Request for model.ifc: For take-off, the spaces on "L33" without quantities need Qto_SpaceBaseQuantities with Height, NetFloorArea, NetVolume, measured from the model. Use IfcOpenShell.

First a look at what the model holds.

```python
import ifcopenshell
import ifcopenshell.util.element
import ifcopenshell.util.unit

model = ifcopenshell.open("model.ifc")
print(model.schema)
for unit_type in ("LENGTHUNIT", "AREAUNIT", "VOLUMEUNIT"):
    print(unit_type, ifcopenshell.util.unit.calculate_unit_scale(model, unit_type))
storey = next(s for s in model.by_type("IfcBuildingStorey") if s.Name == "L33")
spaces = [e for e in ifcopenshell.util.element.get_decomposition(storey) if e.is_a("IfcSpace")]
for e in sorted(spaces, key=lambda e: e.id()):
    print(e.id(), e.is_a(), e.Name, list(ifcopenshell.util.element.get_psets(e, qtos_only=True)), sep=" | ")
```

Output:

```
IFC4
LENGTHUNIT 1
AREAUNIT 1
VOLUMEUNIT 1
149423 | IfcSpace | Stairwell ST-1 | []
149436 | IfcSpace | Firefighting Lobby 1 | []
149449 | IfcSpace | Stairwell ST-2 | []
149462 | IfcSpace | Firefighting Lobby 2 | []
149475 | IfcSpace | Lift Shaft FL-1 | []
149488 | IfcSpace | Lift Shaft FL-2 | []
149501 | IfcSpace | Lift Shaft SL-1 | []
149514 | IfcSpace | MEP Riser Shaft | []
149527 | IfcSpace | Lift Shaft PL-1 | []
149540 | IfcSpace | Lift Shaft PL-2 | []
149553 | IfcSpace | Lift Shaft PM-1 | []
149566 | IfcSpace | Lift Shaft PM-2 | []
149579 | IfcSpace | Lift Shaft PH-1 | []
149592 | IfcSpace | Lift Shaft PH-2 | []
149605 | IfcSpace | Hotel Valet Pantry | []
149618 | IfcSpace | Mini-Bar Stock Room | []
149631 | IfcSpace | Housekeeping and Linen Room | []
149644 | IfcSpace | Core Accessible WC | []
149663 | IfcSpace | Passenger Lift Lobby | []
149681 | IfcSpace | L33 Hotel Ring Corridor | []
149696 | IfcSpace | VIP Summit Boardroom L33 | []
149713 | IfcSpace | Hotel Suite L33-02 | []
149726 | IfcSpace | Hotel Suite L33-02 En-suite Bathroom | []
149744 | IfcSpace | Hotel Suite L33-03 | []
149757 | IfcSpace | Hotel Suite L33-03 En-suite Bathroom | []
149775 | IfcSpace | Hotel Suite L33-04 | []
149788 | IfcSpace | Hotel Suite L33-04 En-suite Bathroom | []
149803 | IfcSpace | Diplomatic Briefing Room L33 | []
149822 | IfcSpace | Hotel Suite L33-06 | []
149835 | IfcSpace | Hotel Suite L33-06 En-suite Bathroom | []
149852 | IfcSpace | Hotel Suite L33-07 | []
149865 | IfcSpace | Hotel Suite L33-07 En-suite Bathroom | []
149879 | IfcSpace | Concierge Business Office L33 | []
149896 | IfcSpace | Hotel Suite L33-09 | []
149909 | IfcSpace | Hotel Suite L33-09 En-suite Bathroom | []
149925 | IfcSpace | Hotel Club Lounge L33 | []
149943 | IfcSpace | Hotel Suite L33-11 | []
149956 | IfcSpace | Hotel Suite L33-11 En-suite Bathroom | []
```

```python
import ifcopenshell
import ifcopenshell.api.pset
import ifcopenshell.geom
import ifcopenshell.util.element
import ifcopenshell.util.shape
import ifcopenshell.util.unit

model = ifcopenshell.open("model.ifc")
unit_scale = ifcopenshell.util.unit.calculate_unit_scale(model)
area_scale = ifcopenshell.util.unit.calculate_unit_scale(model, "AREAUNIT")
volume_scale = ifcopenshell.util.unit.calculate_unit_scale(model, "VOLUMEUNIT")
settings = ifcopenshell.geom.settings()

storey = next(s for s in model.by_type("IfcBuildingStorey") if s.Name == "L33")
spaces = [e for e in ifcopenshell.util.element.get_decomposition(storey) if e.is_a("IfcSpace")]

for e in sorted(spaces, key=lambda e: e.id()):
    if ifcopenshell.util.element.get_psets(e, qtos_only=True, should_inherit=False):
        continue
    # Geometry comes back in metres, in the element's own axes.
    shape = ifcopenshell.geom.create_shape(settings, e)
    values = {
        "Height": ifcopenshell.util.shape.get_z(shape.geometry) / unit_scale,
        "NetFloorArea": ifcopenshell.util.shape.get_footprint_area(shape.geometry) / area_scale,
        "NetVolume": ifcopenshell.util.shape.get_volume(shape.geometry) / volume_scale,
    }
    qto = ifcopenshell.api.pset.add_qto(model, product=e, name="Qto_SpaceBaseQuantities")
    ifcopenshell.api.pset.edit_qto(model, qto=qto, properties=values)
    print(e.id(), {k: round(v, 3) for k, v in values.items()})

model.write("model-out.ifc")
```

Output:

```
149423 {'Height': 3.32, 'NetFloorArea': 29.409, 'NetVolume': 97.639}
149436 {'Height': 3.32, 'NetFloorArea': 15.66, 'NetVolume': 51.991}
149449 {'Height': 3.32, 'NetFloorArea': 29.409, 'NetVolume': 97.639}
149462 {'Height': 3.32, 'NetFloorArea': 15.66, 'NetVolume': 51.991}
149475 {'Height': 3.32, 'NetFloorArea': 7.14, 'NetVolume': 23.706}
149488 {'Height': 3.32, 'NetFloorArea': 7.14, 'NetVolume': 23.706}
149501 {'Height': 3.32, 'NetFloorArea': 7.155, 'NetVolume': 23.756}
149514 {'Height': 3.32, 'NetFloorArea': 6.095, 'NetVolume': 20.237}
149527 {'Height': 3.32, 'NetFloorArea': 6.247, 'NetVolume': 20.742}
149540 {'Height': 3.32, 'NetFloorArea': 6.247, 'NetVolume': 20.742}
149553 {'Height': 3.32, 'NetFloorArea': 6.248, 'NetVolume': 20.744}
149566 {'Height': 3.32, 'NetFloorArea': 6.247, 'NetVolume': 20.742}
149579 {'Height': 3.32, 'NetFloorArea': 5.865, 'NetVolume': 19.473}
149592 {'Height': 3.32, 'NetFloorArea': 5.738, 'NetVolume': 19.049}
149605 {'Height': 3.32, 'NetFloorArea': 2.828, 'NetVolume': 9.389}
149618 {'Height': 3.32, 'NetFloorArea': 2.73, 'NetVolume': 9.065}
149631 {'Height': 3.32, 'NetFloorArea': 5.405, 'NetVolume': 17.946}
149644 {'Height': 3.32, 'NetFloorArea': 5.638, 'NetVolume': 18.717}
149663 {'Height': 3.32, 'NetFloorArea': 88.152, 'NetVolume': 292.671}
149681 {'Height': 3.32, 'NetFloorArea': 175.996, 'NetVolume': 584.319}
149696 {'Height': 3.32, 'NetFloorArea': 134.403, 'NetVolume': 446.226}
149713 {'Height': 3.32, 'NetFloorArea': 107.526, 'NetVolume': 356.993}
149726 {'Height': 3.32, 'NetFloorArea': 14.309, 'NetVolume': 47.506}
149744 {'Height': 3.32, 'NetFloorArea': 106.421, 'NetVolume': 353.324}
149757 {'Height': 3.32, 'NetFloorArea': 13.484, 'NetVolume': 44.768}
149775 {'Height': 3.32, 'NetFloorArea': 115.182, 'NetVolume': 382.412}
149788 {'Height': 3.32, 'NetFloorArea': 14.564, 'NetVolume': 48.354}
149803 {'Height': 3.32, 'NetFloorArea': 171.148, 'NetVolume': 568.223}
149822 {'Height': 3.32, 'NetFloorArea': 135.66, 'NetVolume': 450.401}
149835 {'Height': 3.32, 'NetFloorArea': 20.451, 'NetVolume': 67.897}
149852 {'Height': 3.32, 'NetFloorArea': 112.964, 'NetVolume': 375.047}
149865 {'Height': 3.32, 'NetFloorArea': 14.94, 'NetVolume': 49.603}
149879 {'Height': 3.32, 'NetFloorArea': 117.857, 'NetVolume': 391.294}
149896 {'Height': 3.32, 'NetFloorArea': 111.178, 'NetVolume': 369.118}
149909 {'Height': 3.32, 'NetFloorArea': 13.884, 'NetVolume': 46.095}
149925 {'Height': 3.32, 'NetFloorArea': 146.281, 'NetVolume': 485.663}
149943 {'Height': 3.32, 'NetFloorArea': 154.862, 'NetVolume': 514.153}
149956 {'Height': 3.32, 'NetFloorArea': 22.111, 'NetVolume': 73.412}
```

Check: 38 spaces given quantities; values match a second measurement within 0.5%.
